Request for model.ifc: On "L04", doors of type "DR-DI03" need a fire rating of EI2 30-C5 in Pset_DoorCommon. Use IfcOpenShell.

First a look at what the model holds.

```python
import ifcopenshell
import ifcopenshell.util.element

model = ifcopenshell.open("model.ifc")
print(model.schema)
storey = next(s for s in model.by_type("IfcBuildingStorey") if s.Name == "L04")
doors = [e for e in ifcopenshell.util.element.get_decomposition(storey) if e.is_a("IfcDoor")]
seen = {}
for e in doors:
    element_type = ifcopenshell.util.element.get_type(e)
    key = (element_type.Name if element_type != e and element_type else None, ifcopenshell.util.element.get_pset(e, "Pset_DoorCommon", "FireRating"))
    seen[key] = seen.get(key, 0) + 1
for (name, value), count in sorted(seen.items(), key=str):
    print(count, "x", name, "|", value)
```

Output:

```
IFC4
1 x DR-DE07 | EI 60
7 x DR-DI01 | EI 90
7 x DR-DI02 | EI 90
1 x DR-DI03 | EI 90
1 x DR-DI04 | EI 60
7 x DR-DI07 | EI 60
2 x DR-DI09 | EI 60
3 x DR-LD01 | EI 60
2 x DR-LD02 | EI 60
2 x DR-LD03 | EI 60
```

```python
import ifcopenshell
import ifcopenshell.api.pset
import ifcopenshell.util.element

model = ifcopenshell.open("model.ifc")

storey = next(s for s in model.by_type("IfcBuildingStorey") if s.Name == "L04")
doors = [e for e in ifcopenshell.util.element.get_decomposition(storey) if e.is_a("IfcDoor")]

count = 0
for e in doors:
    element_type = ifcopenshell.util.element.get_type(e)
    if element_type in (None, e) or element_type.Name != "DR-DI03":
        continue
    # add_pset returns the element's existing set when there is one.
    pset = ifcopenshell.api.pset.add_pset(model, product=e, name="Pset_DoorCommon")
    ifcopenshell.api.pset.edit_pset(model, pset=pset, properties={"FireRating": "EI2 30-C5"})
    count += 1

print(count, "doors updated")

model.write("model-out.ifc")
```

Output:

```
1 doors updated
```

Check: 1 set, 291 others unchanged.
